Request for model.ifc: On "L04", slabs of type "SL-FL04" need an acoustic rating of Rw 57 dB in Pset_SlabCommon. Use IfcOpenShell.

First a look at what the model holds.

```python
import ifcopenshell
import ifcopenshell.util.element

model = ifcopenshell.open("model.ifc")
print(model.schema)
storey = next(s for s in model.by_type("IfcBuildingStorey") if s.Name == "L04")
slabs = [e for e in ifcopenshell.util.element.get_decomposition(storey) if e.is_a("IfcSlab")]
seen = {}
for e in slabs:
    element_type = ifcopenshell.util.element.get_type(e)
    key = (element_type.Name if element_type != e and element_type else None, ifcopenshell.util.element.get_pset(e, "Pset_SlabCommon", "AcousticRating"))
    seen[key] = seen.get(key, 0) + 1
for (name, value), count in sorted(seen.items(), key=str):
    print(count, "x", name, "|", value)
```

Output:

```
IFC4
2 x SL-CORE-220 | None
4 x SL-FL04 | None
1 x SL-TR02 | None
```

```python
import ifcopenshell
import ifcopenshell.api.pset
import ifcopenshell.util.element

model = ifcopenshell.open("model.ifc")

storey = next(s for s in model.by_type("IfcBuildingStorey") if s.Name == "L04")
slabs = [e for e in ifcopenshell.util.element.get_decomposition(storey) if e.is_a("IfcSlab")]

count = 0
for e in slabs:
    element_type = ifcopenshell.util.element.get_type(e)
    if element_type in (None, e) or element_type.Name != "SL-FL04":
        continue
    # add_pset returns the element's existing set when there is one.
    pset = ifcopenshell.api.pset.add_pset(model, product=e, name="Pset_SlabCommon")
    ifcopenshell.api.pset.edit_pset(model, pset=pset, properties={"AcousticRating": "Rw 57 dB"})
    count += 1

print(count, "slabs updated")

model.write("model_v2.ifc")
```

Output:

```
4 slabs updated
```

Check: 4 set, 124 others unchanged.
